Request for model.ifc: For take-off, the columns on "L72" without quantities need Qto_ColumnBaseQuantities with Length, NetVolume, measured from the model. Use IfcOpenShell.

First a look at what the model holds.

```python
import ifcopenshell
import ifcopenshell.util.element
import ifcopenshell.util.unit

model = ifcopenshell.open("model.ifc")
print(model.schema)
for unit_type in ("LENGTHUNIT", "AREAUNIT", "VOLUMEUNIT"):
    print(unit_type, ifcopenshell.util.unit.calculate_unit_scale(model, unit_type))
storey = next(s for s in model.by_type("IfcBuildingStorey") if s.Name == "L72")
columns = [e for e in ifcopenshell.util.element.get_decomposition(storey) if e.is_a("IfcColumn")]
for e in sorted(columns, key=lambda e: e.id()):
    print(e.id(), e.is_a(), e.Name, list(ifcopenshell.util.element.get_psets(e, qtos_only=True)), sep=" | ")
```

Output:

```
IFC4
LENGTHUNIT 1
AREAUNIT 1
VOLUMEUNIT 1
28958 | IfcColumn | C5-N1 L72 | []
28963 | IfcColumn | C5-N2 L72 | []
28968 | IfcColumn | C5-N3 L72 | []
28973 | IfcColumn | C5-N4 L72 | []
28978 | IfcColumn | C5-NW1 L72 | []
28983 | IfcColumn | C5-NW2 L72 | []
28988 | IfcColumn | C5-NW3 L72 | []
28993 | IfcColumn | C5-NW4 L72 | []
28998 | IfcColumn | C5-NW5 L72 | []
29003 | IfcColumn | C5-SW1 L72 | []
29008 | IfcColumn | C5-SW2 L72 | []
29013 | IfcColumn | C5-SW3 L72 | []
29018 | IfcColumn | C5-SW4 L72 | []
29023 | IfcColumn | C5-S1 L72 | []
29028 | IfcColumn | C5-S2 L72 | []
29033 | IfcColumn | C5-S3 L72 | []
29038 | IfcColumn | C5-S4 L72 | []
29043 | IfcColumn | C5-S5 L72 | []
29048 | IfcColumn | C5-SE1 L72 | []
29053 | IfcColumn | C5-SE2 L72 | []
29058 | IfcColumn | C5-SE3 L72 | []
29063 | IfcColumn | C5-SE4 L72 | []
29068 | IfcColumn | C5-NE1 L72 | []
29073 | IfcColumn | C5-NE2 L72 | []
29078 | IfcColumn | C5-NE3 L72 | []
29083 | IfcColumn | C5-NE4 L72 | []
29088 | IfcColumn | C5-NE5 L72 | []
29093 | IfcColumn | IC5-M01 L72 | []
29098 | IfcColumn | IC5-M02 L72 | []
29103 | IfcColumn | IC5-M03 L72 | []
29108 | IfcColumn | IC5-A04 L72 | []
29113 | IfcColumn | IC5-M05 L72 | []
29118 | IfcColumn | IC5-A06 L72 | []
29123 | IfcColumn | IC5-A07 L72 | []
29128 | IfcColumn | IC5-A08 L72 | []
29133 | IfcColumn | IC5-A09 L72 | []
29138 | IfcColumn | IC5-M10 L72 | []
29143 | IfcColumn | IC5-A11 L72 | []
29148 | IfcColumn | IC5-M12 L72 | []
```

```python
import ifcopenshell
import ifcopenshell.api.pset
import ifcopenshell.geom
import ifcopenshell.util.element
import ifcopenshell.util.shape
import ifcopenshell.util.unit

model = ifcopenshell.open("model.ifc")
unit_scale = ifcopenshell.util.unit.calculate_unit_scale(model)
volume_scale = ifcopenshell.util.unit.calculate_unit_scale(model, "VOLUMEUNIT")
settings = ifcopenshell.geom.settings()

storey = next(s for s in model.by_type("IfcBuildingStorey") if s.Name == "L72")
columns = [e for e in ifcopenshell.util.element.get_decomposition(storey) if e.is_a("IfcColumn")]

for e in sorted(columns, key=lambda e: e.id()):
    if ifcopenshell.util.element.get_psets(e, qtos_only=True, should_inherit=False):
        continue
    # Geometry comes back in metres, in the element's own axes.
    shape = ifcopenshell.geom.create_shape(settings, e)
    values = {
        "Length": ifcopenshell.util.shape.get_z(shape.geometry) / unit_scale,
        "NetVolume": ifcopenshell.util.shape.get_volume(shape.geometry) / volume_scale,
    }
    qto = ifcopenshell.api.pset.add_qto(model, product=e, name="Qto_ColumnBaseQuantities")
    ifcopenshell.api.pset.edit_qto(model, qto=qto, properties=values)
    print(e.id(), {k: round(v, 3) for k, v in values.items()})

model.write("model_edited.ifc")
```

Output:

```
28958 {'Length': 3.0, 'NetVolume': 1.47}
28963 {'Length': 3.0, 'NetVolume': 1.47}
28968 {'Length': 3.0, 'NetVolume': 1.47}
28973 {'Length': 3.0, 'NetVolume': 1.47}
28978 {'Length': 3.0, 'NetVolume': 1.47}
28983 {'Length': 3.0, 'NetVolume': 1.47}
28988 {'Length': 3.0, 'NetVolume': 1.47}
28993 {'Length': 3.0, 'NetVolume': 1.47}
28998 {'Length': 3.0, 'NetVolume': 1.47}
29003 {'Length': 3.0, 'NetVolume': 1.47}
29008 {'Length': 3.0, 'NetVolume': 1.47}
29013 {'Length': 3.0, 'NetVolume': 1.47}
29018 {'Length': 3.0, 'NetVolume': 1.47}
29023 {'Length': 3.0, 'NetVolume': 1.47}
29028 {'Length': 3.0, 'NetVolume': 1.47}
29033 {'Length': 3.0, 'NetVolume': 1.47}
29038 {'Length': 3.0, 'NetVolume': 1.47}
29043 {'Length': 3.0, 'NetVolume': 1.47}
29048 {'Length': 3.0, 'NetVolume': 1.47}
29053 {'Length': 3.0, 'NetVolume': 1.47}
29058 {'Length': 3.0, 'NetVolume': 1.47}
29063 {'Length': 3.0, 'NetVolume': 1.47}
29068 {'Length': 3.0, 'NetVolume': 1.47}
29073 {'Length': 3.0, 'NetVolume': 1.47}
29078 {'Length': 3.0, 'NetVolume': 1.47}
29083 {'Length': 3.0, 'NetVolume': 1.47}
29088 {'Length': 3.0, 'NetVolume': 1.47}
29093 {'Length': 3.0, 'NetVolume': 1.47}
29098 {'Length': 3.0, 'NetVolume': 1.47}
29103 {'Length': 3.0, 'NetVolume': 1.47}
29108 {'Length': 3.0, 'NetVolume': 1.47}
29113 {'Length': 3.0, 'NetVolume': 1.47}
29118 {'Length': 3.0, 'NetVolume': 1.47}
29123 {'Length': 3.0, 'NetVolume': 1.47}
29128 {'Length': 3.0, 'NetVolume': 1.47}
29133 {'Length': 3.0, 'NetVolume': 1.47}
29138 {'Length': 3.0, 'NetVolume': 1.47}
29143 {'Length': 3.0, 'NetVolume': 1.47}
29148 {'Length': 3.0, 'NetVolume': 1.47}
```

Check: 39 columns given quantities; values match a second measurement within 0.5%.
